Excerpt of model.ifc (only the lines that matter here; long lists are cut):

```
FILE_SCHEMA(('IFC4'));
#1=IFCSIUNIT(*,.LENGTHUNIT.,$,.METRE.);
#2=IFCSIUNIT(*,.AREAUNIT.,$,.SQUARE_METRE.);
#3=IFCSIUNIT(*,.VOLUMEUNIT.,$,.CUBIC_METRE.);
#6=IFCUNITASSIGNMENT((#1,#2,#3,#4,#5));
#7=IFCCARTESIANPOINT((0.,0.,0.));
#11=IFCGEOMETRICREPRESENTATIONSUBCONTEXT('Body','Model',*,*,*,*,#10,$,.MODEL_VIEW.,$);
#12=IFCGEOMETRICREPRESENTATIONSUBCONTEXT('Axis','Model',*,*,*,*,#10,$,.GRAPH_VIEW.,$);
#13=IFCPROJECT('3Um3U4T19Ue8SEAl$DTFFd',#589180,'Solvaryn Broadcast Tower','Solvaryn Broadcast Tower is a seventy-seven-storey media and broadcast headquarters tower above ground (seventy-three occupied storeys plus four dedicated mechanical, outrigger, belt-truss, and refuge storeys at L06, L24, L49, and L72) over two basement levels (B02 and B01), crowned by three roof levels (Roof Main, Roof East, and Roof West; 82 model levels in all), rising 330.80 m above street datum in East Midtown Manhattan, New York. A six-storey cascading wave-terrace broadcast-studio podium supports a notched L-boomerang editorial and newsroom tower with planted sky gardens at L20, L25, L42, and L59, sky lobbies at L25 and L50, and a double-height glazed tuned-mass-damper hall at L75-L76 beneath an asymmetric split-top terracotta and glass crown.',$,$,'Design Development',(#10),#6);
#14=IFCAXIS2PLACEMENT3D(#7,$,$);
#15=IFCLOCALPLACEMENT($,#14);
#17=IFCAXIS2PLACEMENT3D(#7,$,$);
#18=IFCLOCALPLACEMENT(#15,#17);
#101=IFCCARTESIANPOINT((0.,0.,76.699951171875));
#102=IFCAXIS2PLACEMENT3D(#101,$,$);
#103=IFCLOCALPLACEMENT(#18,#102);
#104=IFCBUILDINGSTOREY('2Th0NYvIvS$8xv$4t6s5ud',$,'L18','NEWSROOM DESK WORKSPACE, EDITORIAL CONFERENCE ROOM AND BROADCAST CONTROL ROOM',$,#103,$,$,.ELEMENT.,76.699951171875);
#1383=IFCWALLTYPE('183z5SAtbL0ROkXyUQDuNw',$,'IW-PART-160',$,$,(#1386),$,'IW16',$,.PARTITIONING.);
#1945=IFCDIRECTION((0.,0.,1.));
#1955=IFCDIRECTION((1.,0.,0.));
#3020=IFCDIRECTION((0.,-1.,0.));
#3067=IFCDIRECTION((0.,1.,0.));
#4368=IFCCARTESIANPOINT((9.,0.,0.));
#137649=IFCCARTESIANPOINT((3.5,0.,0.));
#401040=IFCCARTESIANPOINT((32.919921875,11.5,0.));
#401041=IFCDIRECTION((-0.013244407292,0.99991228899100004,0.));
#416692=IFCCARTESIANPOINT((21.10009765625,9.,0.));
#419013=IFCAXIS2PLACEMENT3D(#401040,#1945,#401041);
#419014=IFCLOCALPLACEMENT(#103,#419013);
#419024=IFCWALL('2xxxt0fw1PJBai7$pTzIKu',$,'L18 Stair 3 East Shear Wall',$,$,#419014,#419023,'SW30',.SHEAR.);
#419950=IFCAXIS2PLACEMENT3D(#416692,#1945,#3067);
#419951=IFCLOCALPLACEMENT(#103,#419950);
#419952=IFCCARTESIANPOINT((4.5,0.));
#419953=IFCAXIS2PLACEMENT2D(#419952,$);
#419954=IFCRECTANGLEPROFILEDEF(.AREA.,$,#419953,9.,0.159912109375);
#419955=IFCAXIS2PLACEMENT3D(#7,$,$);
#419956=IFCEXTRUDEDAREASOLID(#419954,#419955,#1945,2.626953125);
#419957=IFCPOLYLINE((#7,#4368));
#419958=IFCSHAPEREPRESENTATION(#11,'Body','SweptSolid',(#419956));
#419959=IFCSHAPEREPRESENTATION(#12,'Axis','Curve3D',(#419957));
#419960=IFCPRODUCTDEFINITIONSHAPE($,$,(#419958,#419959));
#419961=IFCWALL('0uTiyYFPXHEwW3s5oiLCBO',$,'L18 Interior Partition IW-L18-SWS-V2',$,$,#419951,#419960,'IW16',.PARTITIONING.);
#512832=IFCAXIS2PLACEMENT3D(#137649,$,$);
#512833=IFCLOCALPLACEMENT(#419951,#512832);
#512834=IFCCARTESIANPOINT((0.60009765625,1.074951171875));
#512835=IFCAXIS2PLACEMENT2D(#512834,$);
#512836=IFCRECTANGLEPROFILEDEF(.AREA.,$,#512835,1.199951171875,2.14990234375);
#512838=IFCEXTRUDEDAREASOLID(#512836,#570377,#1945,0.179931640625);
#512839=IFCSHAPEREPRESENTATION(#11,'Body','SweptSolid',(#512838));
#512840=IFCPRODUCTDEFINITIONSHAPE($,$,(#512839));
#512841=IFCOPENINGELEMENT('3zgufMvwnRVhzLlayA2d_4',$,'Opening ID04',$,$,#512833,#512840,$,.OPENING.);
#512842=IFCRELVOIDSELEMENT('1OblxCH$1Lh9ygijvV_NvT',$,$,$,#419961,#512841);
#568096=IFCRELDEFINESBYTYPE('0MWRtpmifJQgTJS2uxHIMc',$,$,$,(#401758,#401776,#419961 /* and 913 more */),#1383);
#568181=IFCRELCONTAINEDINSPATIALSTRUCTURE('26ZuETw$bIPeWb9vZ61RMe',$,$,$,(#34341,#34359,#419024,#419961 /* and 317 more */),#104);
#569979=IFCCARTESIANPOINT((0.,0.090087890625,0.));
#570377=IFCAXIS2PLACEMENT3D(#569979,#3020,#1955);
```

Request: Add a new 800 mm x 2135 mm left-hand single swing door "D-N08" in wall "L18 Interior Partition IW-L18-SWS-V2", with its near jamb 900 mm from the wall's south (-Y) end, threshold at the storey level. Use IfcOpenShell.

```python
import numpy as np
import ifcopenshell
import ifcopenshell.api.feature
import ifcopenshell.api.geometry
import ifcopenshell.api.root
import ifcopenshell.api.spatial
import ifcopenshell.geom
import ifcopenshell.util.element
import ifcopenshell.util.placement
import ifcopenshell.util.representation
import ifcopenshell.util.shape
import ifcopenshell.util.unit

model = ifcopenshell.open("model.ifc")
unit_scale = ifcopenshell.util.unit.calculate_unit_scale(model)
settings = ifcopenshell.geom.settings()


def volume(element):
    """Net volume in cubic metres, openings subtracted."""
    shape = ifcopenshell.geom.create_shape(settings, element)
    return ifcopenshell.util.shape.get_volume(shape.geometry)


wall = model.by_id(419961)
storey = ifcopenshell.util.element.get_container(wall, ifc_class="IfcBuildingStorey")
context = ifcopenshell.util.representation.get_context(model, "Model", "Body", "MODEL_VIEW")
before = volume(wall)

width, height, from_end, sill = 0.8, 2.135, 0.9, 0.0  # metres

# The wall runs along its own X axis, and the end named is its -X end.
wall_shape = ifcopenshell.geom.create_shape(settings, wall)
x, y, z = ifcopenshell.util.shape.get_vertices(wall_shape.geometry).T
start = x.min() + from_end
face, thickness = float(y.min()), float(y.max() - y.min())
wall_matrix = ifcopenshell.util.placement.get_local_placement(wall.ObjectPlacement)
level = ifcopenshell.util.placement.get_local_placement(storey.ObjectPlacement)[2, 3]


def in_wall(x, y):
    """Placement at x, y metres in the wall's axes, at sill height."""
    matrix = wall_matrix.copy()
    matrix[:, 3] = wall_matrix @ np.array([x / unit_scale, y / unit_scale, 0.0, 1.0])
    matrix[2, 3] = level + sill / unit_scale
    return matrix


# Opening: a box that overshoots both wall faces by 50 mm.
opening = ifcopenshell.api.root.create_entity(model, ifc_class="IfcOpeningElement", predefined_type="OPENING")
box = ifcopenshell.api.geometry.add_wall_representation(
    model, context=context, length=width, height=height, thickness=thickness + 0.1
)
ifcopenshell.api.geometry.assign_representation(model, product=opening, representation=box)
ifcopenshell.api.geometry.edit_object_placement(model, product=opening, matrix=in_wall(start, face - 0.05), is_si=False)
ifcopenshell.api.feature.add_feature(model, feature=opening, element=wall)

door = ifcopenshell.api.root.create_entity(model, ifc_class="IfcDoor", name="D-N08", predefined_type="DOOR")
door.OverallWidth, door.OverallHeight = width / unit_scale, height / unit_scale
door.OperationType = "SINGLE_SWING_LEFT"
body = ifcopenshell.api.geometry.add_door_representation(
    model,
    context=context,
    overall_width=door.OverallWidth,
    overall_height=door.OverallHeight,
    operation_type="SINGLE_SWING_LEFT",
    lining_properties={"LiningDepth": thickness / unit_scale, "ThresholdDepth": thickness / unit_scale},
)
ifcopenshell.api.geometry.assign_representation(model, product=door, representation=body)
ifcopenshell.api.spatial.assign_container(model, products=[door], relating_structure=storey)
ifcopenshell.api.feature.add_filling(model, opening=opening, element=door)

# The lining spans the wall, so the door starts at the wall face.
ifcopenshell.api.geometry.edit_object_placement(model, product=door, matrix=in_wall(start, face), is_si=False)

after = volume(wall)

print(f"wall volume {before:.3f} -> {after:.3f} m3")

model.write("model_updated.ifc")
```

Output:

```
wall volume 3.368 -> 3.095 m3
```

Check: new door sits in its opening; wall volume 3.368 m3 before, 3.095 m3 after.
